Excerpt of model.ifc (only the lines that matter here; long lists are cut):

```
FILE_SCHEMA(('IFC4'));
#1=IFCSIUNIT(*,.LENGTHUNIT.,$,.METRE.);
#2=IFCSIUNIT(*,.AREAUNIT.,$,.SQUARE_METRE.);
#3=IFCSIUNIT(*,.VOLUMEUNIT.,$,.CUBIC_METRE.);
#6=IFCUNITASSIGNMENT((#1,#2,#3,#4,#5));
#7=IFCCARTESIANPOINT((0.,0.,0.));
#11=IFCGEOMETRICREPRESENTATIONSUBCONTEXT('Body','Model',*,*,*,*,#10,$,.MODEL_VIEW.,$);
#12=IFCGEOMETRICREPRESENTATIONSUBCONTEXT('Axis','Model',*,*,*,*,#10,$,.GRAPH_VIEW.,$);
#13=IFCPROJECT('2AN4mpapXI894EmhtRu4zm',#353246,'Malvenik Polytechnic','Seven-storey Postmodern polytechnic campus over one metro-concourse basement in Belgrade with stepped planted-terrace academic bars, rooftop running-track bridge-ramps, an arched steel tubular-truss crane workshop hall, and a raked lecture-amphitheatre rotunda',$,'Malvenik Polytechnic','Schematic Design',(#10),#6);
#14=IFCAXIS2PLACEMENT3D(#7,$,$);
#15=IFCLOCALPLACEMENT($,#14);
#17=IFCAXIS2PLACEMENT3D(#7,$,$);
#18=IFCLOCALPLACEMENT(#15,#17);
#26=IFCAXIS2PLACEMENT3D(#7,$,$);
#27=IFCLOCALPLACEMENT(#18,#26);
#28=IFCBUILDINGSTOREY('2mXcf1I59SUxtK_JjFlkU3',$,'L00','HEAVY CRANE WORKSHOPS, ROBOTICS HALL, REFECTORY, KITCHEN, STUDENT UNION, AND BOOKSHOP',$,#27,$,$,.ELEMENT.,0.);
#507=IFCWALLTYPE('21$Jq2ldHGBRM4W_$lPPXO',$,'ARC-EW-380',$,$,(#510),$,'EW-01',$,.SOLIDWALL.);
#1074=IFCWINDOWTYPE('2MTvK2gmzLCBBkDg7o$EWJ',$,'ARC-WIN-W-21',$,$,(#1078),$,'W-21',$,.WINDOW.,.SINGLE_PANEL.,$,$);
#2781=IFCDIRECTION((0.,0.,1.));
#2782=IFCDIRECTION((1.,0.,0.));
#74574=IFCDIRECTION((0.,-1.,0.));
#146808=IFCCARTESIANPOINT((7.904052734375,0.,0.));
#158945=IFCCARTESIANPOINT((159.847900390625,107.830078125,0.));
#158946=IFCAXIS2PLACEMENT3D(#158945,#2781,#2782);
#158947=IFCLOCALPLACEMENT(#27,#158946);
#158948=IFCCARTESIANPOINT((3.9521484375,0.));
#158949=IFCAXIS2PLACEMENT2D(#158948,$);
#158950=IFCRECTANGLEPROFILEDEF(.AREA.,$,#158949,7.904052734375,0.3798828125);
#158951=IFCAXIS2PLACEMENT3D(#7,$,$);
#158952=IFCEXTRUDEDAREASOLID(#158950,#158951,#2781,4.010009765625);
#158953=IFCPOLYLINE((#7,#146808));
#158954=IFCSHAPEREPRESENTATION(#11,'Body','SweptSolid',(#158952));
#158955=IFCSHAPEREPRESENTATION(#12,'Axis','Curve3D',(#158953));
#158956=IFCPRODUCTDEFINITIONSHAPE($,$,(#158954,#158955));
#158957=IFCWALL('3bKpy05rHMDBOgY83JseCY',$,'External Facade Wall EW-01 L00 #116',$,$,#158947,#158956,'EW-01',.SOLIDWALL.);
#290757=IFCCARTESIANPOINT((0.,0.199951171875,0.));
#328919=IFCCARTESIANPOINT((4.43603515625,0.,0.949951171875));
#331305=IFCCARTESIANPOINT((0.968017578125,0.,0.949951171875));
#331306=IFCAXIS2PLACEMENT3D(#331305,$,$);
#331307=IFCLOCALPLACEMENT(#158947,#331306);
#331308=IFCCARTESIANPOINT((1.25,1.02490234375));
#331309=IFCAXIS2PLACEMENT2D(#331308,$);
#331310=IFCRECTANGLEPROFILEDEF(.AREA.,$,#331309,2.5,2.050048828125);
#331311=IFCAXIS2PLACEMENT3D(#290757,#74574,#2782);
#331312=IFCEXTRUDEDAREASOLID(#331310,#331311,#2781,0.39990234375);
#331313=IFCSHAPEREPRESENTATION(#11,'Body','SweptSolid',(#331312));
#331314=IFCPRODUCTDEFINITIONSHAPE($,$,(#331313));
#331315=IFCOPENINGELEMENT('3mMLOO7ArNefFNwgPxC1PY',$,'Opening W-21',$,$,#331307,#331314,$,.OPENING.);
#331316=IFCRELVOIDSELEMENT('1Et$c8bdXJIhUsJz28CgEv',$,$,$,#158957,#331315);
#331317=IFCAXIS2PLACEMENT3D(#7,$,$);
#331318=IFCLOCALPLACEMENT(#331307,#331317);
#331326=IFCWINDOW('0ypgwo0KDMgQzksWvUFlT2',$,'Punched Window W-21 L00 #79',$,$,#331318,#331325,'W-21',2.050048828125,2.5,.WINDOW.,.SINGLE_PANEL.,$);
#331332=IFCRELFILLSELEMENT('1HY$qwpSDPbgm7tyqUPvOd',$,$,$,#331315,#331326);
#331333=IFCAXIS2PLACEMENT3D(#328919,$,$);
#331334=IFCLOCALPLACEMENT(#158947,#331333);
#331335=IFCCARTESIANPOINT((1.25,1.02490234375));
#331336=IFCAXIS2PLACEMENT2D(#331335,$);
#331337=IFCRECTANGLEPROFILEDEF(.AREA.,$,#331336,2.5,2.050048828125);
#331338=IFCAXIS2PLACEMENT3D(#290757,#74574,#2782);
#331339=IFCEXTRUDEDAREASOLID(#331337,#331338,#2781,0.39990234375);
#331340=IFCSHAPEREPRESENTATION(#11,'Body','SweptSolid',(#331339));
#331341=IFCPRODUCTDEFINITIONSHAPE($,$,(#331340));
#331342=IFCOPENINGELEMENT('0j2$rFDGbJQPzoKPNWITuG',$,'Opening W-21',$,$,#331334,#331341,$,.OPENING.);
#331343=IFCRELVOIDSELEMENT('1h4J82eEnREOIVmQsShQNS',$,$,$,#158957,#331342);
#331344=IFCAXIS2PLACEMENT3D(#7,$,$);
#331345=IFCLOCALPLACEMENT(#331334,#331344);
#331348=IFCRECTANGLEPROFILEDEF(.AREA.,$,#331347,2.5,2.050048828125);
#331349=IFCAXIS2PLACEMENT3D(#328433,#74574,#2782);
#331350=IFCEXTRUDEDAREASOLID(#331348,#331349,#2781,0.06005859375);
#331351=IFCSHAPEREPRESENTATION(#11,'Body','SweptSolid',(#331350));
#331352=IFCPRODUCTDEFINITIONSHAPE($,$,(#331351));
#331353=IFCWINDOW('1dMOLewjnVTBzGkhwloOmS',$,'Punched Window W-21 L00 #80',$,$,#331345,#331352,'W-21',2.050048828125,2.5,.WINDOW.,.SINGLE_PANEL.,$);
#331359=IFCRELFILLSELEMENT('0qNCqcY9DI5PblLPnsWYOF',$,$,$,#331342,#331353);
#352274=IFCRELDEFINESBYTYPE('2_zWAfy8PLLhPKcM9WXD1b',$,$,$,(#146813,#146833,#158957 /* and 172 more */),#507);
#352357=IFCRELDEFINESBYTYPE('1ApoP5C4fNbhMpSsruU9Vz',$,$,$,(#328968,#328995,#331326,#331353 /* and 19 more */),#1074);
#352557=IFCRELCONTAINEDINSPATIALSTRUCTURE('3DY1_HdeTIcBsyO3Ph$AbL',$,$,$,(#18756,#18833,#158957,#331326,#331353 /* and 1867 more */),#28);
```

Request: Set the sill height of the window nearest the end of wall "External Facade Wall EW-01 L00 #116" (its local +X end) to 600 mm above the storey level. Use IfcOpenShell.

```python
import numpy as np
import ifcopenshell
import ifcopenshell.api.geometry
import ifcopenshell.geom
import ifcopenshell.util.element
import ifcopenshell.util.placement
import ifcopenshell.util.shape
import ifcopenshell.util.unit

model = ifcopenshell.open("model.ifc")
unit_scale = ifcopenshell.util.unit.calculate_unit_scale(model)

window = model.by_guid("1dMOLewjnVTBzGkhwloOmS")
opening = window.FillsVoids[0].RelatingOpeningElement
storey = ifcopenshell.util.element.get_container(window, ifc_class="IfcBuildingStorey")
level = ifcopenshell.util.placement.get_local_placement(storey.ObjectPlacement)[2, 3]

# The opening's origin need not be at the sill, so measure its lowest point.
shape = ifcopenshell.geom.create_shape(ifcopenshell.geom.settings(), opening)
bottom = ifcopenshell.util.shape.get_shape_bottom_elevation(shape, shape.geometry) / unit_scale
dz = level + 0.6 - bottom

shift = np.array([0.0, 0.0, dz])
# The window is placed relative to its opening, so it follows when the opening moves.
matrix = ifcopenshell.util.placement.get_local_placement(opening.ObjectPlacement)
matrix[:3, 3] += shift
ifcopenshell.api.geometry.edit_object_placement(
    model, product=opening, matrix=matrix, is_si=False, should_transform_children=True
)

print(f"moved by {dz * unit_scale:+.3f} m")

model.write("model_updated.ifc")
```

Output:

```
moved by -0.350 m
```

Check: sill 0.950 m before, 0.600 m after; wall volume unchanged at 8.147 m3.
